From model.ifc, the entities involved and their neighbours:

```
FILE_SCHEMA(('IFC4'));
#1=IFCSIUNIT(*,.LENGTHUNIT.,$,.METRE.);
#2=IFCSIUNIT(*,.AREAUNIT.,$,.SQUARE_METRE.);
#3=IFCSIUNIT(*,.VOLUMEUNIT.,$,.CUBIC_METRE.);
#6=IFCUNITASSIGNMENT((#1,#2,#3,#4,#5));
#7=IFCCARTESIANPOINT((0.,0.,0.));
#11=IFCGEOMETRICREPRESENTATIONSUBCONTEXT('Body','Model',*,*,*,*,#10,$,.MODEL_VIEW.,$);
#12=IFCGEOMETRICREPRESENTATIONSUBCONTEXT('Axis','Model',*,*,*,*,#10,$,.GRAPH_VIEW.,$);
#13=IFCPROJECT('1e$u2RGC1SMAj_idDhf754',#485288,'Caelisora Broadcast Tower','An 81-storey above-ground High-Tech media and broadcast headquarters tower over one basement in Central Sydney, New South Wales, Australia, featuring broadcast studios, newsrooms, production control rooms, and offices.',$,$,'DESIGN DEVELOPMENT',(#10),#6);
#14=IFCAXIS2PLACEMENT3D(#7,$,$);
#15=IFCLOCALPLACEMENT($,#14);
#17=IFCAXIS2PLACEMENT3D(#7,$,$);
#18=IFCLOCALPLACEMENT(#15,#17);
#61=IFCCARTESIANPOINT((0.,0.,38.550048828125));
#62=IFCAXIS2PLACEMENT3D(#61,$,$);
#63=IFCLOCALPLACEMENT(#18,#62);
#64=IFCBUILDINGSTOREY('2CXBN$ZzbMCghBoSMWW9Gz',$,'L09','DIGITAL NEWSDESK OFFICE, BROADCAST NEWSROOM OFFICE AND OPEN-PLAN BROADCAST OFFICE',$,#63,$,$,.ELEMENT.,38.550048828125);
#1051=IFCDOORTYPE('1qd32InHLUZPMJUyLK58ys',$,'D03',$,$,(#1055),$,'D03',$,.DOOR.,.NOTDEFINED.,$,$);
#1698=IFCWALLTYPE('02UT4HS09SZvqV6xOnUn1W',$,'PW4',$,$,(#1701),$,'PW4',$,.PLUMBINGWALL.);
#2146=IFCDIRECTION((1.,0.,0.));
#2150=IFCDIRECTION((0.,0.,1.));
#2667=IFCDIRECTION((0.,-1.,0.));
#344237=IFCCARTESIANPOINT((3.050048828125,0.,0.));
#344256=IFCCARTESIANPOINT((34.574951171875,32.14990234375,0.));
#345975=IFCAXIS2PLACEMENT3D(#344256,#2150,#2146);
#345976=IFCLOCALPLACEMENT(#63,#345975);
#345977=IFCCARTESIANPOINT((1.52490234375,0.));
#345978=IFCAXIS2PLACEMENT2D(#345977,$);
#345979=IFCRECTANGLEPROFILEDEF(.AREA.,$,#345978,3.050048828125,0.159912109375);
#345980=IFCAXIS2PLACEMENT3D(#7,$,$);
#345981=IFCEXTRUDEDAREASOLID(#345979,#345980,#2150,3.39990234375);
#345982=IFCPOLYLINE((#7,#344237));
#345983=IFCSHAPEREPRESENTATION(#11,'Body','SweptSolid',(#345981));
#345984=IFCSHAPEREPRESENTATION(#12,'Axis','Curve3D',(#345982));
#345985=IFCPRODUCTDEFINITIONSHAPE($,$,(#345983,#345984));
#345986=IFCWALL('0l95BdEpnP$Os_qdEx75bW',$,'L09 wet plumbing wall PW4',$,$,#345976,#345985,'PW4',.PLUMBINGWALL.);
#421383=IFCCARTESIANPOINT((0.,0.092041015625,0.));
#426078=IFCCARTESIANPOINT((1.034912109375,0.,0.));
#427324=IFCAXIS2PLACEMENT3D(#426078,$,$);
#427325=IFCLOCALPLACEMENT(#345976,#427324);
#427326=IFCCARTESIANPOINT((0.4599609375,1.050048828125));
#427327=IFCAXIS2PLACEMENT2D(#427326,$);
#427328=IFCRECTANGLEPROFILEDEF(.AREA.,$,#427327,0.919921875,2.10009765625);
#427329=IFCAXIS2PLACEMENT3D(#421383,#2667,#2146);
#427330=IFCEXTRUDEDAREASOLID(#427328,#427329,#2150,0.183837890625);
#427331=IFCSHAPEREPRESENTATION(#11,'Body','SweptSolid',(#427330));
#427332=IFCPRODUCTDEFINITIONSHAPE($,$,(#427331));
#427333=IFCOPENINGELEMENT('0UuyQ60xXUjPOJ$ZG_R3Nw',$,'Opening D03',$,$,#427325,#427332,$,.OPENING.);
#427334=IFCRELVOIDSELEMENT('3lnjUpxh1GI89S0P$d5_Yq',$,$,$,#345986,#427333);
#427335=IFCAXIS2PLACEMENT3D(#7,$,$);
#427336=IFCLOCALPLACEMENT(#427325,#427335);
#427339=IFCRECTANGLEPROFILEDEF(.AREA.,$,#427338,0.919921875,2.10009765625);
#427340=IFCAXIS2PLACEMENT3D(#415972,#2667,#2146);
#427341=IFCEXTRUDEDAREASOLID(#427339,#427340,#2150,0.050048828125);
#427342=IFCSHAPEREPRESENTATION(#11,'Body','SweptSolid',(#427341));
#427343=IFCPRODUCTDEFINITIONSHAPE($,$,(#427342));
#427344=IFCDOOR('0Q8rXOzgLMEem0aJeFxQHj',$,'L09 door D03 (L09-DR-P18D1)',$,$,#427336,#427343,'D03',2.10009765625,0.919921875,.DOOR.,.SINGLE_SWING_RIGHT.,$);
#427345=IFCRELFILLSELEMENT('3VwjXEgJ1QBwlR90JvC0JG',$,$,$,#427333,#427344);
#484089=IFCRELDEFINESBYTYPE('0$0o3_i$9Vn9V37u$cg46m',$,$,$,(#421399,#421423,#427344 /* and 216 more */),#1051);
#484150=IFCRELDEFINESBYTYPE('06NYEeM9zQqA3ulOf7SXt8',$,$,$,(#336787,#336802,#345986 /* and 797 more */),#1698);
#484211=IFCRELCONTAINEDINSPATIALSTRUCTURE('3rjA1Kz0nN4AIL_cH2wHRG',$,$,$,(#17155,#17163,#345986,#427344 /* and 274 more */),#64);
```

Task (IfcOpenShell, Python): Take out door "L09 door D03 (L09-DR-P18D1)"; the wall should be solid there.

```python
import ifcopenshell
import ifcopenshell.api.feature
import ifcopenshell.api.root
import ifcopenshell.geom
import ifcopenshell.util.shape

model = ifcopenshell.open("model.ifc")
settings = ifcopenshell.geom.settings()


def volume(element):
    """Net volume in cubic metres, openings subtracted."""
    shape = ifcopenshell.geom.create_shape(settings, element)
    return ifcopenshell.util.shape.get_volume(shape.geometry)


door = model.by_guid("0Q8rXOzgLMEem0aJeFxQHj")
opening = door.FillsVoids[0].RelatingOpeningElement
wall = opening.VoidsElements[0].RelatingBuildingElement
before = volume(wall)

ifcopenshell.api.root.remove_product(model, product=door)
ifcopenshell.api.feature.remove_feature(model, feature=opening)

after = volume(wall)

print(f"wall volume {before:.3f} -> {after:.3f} m3")

model.write("model-out.ifc")
```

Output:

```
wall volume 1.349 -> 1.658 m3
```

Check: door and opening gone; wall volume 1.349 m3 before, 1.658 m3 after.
